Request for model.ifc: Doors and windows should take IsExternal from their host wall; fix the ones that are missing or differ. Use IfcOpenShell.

First a look at what the model holds.

```python
import ifcopenshell
import ifcopenshell.util.element

model = ifcopenshell.open("model.ifc")
print(model.schema)
seen = {}
for e in model.by_type("IfcDoor") + model.by_type("IfcWindow"):
    if not e.FillsVoids:
        continue
    host = e.FillsVoids[0].RelatingOpeningElement.VoidsElements[0].RelatingBuildingElement
    own = ifcopenshell.util.element.get_pset(e, f"Pset_{e.is_a()[3:].removesuffix('StandardCase')}Common", "IsExternal")
    wall = ifcopenshell.util.element.get_pset(host, "Pset_WallCommon", "IsExternal")
    seen[e.is_a(), own, wall] = seen.get((e.is_a(), own, wall), 0) + 1
for (cls, own, wall), count in sorted(seen.items(), key=str):
    print(count, cls, "IsExternal:", own, "| host wall:", wall)
```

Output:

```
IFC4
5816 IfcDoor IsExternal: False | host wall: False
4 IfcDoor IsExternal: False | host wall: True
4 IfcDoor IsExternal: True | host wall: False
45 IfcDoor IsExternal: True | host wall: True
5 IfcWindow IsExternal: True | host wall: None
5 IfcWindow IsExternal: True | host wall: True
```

```python
import ifcopenshell
import ifcopenshell.api.pset
import ifcopenshell.util.element

model = ifcopenshell.open("model.ifc")

count = 0
for ifc_class, pset_name in (("IfcDoor", "Pset_DoorCommon"), ("IfcWindow", "Pset_WindowCommon")):
    for e in model.by_type(ifc_class):
        if not e.FillsVoids:
            continue
        host = e.FillsVoids[0].RelatingOpeningElement.VoidsElements[0].RelatingBuildingElement
        external = ifcopenshell.util.element.get_pset(host, "Pset_WallCommon", "IsExternal")
        if external is None or ifcopenshell.util.element.get_pset(e, pset_name, "IsExternal") == external:
            continue
        pset = ifcopenshell.api.pset.add_pset(model, product=e, name=pset_name)
        ifcopenshell.api.pset.edit_pset(model, pset=pset, properties={"IsExternal": external})
        count += 1

print(count, "updated")

model.write("model_v2.ifc")
```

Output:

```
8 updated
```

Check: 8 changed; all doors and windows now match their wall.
